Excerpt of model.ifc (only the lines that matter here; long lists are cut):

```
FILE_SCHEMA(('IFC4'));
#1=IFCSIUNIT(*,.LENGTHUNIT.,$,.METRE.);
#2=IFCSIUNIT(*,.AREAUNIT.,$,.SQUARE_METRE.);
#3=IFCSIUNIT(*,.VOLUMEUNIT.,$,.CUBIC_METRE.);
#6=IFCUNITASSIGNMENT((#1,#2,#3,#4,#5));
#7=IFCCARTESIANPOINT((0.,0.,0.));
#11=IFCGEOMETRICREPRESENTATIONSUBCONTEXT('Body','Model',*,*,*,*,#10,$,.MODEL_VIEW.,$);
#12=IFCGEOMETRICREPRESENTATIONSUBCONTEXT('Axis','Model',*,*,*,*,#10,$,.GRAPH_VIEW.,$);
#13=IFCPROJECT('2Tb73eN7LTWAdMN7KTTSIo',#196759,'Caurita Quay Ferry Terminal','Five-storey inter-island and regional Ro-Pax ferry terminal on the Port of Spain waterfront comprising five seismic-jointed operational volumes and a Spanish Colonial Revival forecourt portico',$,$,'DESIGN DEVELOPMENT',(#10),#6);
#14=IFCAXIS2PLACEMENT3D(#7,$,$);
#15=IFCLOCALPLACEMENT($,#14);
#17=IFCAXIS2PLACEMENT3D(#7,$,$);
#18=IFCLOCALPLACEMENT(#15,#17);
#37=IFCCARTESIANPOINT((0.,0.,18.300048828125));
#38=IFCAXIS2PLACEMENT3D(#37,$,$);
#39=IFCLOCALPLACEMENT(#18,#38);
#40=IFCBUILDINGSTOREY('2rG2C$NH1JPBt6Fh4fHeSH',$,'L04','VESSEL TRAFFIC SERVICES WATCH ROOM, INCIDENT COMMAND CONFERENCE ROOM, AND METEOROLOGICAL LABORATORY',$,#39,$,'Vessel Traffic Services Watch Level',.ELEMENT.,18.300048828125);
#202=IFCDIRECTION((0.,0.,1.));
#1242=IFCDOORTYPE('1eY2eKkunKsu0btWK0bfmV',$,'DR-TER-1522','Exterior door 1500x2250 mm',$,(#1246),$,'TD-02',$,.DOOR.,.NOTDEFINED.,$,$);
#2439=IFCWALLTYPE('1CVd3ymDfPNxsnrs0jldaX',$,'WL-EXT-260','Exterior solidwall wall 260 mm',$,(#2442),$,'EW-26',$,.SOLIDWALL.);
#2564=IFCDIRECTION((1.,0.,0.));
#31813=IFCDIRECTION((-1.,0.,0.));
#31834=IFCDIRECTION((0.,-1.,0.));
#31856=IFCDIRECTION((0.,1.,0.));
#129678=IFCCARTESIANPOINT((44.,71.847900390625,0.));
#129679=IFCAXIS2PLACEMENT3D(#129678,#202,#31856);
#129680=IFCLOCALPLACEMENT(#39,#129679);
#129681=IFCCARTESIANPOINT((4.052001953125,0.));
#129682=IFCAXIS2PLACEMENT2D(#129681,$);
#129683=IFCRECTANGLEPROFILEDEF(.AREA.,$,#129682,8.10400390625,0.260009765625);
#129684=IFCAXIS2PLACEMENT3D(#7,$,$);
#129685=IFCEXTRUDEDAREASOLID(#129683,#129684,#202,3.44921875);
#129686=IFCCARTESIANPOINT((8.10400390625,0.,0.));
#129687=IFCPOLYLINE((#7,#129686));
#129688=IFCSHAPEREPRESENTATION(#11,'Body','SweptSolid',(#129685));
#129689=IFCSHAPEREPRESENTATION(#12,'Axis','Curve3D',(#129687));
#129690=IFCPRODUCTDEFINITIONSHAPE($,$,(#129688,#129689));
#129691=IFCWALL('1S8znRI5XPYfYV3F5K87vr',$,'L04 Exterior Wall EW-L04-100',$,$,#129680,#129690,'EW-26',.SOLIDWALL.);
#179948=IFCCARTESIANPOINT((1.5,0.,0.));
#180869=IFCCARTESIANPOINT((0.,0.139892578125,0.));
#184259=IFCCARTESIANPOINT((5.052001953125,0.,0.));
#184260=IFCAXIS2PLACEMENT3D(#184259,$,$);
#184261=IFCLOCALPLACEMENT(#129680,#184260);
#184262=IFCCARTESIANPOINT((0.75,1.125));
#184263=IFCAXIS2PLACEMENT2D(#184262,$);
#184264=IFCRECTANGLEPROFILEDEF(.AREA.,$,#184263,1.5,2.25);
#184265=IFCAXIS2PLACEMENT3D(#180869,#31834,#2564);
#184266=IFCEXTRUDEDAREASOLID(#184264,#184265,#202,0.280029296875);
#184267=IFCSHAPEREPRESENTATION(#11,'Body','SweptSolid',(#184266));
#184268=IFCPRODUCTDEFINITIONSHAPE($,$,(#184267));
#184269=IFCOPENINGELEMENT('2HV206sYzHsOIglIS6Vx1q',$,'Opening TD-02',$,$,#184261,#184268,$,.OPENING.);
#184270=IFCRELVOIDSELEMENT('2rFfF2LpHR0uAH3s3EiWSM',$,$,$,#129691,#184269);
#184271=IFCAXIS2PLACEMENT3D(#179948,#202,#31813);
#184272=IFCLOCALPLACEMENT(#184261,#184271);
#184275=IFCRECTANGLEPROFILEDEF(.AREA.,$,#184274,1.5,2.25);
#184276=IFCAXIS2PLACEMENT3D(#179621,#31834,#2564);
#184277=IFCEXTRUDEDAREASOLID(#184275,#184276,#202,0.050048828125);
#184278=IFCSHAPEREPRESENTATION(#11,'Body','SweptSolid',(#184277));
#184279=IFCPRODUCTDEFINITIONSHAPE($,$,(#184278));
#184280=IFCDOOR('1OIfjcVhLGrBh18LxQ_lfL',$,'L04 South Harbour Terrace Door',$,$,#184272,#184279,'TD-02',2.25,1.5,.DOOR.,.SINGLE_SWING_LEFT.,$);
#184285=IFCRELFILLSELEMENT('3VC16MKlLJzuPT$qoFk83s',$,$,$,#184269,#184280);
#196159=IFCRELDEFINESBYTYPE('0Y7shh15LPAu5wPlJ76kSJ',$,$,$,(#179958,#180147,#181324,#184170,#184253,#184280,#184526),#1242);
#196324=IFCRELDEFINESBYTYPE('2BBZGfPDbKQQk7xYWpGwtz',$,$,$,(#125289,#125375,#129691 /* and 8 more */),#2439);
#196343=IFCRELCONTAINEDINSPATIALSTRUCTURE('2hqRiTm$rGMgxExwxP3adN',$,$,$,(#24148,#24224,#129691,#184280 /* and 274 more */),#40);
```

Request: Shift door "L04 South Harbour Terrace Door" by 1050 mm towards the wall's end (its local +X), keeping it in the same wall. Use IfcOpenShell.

```python
import ifcopenshell
import ifcopenshell.api.geometry
import ifcopenshell.util.placement

model = ifcopenshell.open("model.ifc")

door = model.by_id(184280)
opening = door.FillsVoids[0].RelatingOpeningElement
wall = opening.VoidsElements[0].RelatingBuildingElement

wall_matrix = ifcopenshell.util.placement.get_local_placement(wall.ObjectPlacement)
shift = wall_matrix[:3, 0] * 1.05
before = ifcopenshell.util.placement.get_local_placement(door.ObjectPlacement)[:3, 3].copy()

# The door is placed relative to its opening, so it follows when the opening moves.
matrix = ifcopenshell.util.placement.get_local_placement(opening.ObjectPlacement)
matrix[:3, 3] += shift
ifcopenshell.api.geometry.edit_object_placement(
    model, product=opening, matrix=matrix, is_si=False, should_transform_children=True
)

after = ifcopenshell.util.placement.get_local_placement(door.ObjectPlacement)[:3, 3]
print("door moved by", (after - before).round(3) + 0.0)

model.write("model_v2.ifc")
```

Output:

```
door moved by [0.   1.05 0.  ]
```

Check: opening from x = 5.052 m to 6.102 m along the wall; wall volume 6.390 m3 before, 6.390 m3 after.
